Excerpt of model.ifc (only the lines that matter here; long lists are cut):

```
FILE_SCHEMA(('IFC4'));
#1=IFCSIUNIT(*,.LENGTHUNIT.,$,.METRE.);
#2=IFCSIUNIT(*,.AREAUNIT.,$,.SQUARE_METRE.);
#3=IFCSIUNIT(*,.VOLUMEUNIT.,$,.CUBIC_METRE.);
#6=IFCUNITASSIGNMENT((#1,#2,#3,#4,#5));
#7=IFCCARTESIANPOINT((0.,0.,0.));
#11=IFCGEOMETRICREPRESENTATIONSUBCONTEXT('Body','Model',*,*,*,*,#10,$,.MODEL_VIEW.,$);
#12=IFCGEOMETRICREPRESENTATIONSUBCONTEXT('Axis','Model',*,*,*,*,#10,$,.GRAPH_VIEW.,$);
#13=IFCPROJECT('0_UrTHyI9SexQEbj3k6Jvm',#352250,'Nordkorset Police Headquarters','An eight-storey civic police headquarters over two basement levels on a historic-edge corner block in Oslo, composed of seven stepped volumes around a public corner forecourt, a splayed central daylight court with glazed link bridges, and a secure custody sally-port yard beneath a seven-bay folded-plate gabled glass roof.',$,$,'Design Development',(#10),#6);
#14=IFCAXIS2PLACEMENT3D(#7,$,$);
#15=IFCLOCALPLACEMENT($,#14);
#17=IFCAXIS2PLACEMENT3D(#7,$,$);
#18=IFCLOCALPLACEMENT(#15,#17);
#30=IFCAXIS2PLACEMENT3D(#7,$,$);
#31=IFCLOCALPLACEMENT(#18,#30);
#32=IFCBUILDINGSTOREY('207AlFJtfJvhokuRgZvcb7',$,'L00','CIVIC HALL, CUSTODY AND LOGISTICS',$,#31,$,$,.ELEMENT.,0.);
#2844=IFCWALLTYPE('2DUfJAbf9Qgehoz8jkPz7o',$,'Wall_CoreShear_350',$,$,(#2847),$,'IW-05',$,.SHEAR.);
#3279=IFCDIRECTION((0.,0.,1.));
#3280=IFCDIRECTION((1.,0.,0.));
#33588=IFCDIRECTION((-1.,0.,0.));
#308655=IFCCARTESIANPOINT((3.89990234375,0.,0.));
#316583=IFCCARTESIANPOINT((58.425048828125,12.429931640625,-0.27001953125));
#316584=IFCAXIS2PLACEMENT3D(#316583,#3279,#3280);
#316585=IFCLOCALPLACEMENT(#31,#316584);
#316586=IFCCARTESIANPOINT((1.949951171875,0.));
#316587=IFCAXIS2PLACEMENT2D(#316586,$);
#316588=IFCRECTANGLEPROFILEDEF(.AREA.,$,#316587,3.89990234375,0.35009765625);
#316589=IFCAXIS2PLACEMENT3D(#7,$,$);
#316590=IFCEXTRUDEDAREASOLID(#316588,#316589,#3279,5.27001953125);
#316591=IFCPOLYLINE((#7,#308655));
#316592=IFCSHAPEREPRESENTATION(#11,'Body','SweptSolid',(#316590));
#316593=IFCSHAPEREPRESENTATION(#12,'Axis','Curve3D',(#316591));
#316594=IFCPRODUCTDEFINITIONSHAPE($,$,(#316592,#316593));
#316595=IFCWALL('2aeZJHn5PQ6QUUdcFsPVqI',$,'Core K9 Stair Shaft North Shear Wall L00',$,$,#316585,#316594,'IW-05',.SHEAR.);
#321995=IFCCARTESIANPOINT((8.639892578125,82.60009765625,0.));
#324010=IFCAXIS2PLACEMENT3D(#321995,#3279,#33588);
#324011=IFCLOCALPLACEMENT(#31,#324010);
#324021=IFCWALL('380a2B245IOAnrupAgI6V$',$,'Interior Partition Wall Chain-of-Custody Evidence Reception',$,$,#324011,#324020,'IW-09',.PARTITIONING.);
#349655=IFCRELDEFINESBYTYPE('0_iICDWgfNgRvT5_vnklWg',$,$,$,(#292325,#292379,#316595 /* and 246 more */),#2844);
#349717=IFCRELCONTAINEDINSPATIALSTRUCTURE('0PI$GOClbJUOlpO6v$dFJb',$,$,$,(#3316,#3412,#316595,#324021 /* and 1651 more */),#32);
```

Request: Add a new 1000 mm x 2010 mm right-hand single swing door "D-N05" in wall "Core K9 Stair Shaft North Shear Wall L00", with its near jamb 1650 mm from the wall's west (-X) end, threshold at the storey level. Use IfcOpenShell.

```python
import numpy as np
import ifcopenshell
import ifcopenshell.api.feature
import ifcopenshell.api.geometry
import ifcopenshell.api.root
import ifcopenshell.api.spatial
import ifcopenshell.geom
import ifcopenshell.util.element
import ifcopenshell.util.placement
import ifcopenshell.util.representation
import ifcopenshell.util.shape
import ifcopenshell.util.unit

model = ifcopenshell.open("model.ifc")
unit_scale = ifcopenshell.util.unit.calculate_unit_scale(model)
settings = ifcopenshell.geom.settings()


def volume(element):
    """Net volume in cubic metres, openings subtracted."""
    shape = ifcopenshell.geom.create_shape(settings, element)
    return ifcopenshell.util.shape.get_volume(shape.geometry)


wall = model.by_guid("2aeZJHn5PQ6QUUdcFsPVqI")
storey = ifcopenshell.util.element.get_container(wall, ifc_class="IfcBuildingStorey")
context = ifcopenshell.util.representation.get_context(model, "Model", "Body", "MODEL_VIEW")
before = volume(wall)

width, height, from_end, sill = 1, 2.01, 1.65, 0.0  # metres

# The wall runs along its own X axis, and the end named is its -X end.
wall_shape = ifcopenshell.geom.create_shape(settings, wall)
x, y, z = ifcopenshell.util.shape.get_vertices(wall_shape.geometry).T
start = x.min() + from_end
face, thickness = float(y.min()), float(y.max() - y.min())
wall_matrix = ifcopenshell.util.placement.get_local_placement(wall.ObjectPlacement)
level = ifcopenshell.util.placement.get_local_placement(storey.ObjectPlacement)[2, 3]


def in_wall(x, y):
    """Placement at x, y metres in the wall's axes, at sill height."""
    matrix = wall_matrix.copy()
    matrix[:, 3] = wall_matrix @ np.array([x / unit_scale, y / unit_scale, 0.0, 1.0])
    matrix[2, 3] = level + sill / unit_scale
    return matrix


# Opening: a box that overshoots both wall faces by 50 mm.
opening = ifcopenshell.api.root.create_entity(model, ifc_class="IfcOpeningElement", predefined_type="OPENING")
box = ifcopenshell.api.geometry.add_wall_representation(
    model, context=context, length=width, height=height, thickness=thickness + 0.1
)
ifcopenshell.api.geometry.assign_representation(model, product=opening, representation=box)
ifcopenshell.api.geometry.edit_object_placement(model, product=opening, matrix=in_wall(start, face - 0.05), is_si=False)
ifcopenshell.api.feature.add_feature(model, feature=opening, element=wall)

door = ifcopenshell.api.root.create_entity(model, ifc_class="IfcDoor", name="D-N05", predefined_type="DOOR")
door.OverallWidth, door.OverallHeight = width / unit_scale, height / unit_scale
door.OperationType = "SINGLE_SWING_RIGHT"
body = ifcopenshell.api.geometry.add_door_representation(
    model,
    context=context,
    overall_width=door.OverallWidth,
    overall_height=door.OverallHeight,
    operation_type="SINGLE_SWING_RIGHT",
    lining_properties={"LiningDepth": thickness / unit_scale, "ThresholdDepth": thickness / unit_scale},
)
ifcopenshell.api.geometry.assign_representation(model, product=door, representation=body)
ifcopenshell.api.spatial.assign_container(model, products=[door], relating_structure=storey)
ifcopenshell.api.feature.add_filling(model, opening=opening, element=door)

# The lining spans the wall, so the door starts at the wall face.
ifcopenshell.api.geometry.edit_object_placement(model, product=door, matrix=in_wall(start, face), is_si=False)

after = volume(wall)

print(f"wall volume {before:.3f} -> {after:.3f} m3")

model.write("model-out.ifc")
```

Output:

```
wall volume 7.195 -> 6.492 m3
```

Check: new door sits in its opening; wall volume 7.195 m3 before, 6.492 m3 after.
